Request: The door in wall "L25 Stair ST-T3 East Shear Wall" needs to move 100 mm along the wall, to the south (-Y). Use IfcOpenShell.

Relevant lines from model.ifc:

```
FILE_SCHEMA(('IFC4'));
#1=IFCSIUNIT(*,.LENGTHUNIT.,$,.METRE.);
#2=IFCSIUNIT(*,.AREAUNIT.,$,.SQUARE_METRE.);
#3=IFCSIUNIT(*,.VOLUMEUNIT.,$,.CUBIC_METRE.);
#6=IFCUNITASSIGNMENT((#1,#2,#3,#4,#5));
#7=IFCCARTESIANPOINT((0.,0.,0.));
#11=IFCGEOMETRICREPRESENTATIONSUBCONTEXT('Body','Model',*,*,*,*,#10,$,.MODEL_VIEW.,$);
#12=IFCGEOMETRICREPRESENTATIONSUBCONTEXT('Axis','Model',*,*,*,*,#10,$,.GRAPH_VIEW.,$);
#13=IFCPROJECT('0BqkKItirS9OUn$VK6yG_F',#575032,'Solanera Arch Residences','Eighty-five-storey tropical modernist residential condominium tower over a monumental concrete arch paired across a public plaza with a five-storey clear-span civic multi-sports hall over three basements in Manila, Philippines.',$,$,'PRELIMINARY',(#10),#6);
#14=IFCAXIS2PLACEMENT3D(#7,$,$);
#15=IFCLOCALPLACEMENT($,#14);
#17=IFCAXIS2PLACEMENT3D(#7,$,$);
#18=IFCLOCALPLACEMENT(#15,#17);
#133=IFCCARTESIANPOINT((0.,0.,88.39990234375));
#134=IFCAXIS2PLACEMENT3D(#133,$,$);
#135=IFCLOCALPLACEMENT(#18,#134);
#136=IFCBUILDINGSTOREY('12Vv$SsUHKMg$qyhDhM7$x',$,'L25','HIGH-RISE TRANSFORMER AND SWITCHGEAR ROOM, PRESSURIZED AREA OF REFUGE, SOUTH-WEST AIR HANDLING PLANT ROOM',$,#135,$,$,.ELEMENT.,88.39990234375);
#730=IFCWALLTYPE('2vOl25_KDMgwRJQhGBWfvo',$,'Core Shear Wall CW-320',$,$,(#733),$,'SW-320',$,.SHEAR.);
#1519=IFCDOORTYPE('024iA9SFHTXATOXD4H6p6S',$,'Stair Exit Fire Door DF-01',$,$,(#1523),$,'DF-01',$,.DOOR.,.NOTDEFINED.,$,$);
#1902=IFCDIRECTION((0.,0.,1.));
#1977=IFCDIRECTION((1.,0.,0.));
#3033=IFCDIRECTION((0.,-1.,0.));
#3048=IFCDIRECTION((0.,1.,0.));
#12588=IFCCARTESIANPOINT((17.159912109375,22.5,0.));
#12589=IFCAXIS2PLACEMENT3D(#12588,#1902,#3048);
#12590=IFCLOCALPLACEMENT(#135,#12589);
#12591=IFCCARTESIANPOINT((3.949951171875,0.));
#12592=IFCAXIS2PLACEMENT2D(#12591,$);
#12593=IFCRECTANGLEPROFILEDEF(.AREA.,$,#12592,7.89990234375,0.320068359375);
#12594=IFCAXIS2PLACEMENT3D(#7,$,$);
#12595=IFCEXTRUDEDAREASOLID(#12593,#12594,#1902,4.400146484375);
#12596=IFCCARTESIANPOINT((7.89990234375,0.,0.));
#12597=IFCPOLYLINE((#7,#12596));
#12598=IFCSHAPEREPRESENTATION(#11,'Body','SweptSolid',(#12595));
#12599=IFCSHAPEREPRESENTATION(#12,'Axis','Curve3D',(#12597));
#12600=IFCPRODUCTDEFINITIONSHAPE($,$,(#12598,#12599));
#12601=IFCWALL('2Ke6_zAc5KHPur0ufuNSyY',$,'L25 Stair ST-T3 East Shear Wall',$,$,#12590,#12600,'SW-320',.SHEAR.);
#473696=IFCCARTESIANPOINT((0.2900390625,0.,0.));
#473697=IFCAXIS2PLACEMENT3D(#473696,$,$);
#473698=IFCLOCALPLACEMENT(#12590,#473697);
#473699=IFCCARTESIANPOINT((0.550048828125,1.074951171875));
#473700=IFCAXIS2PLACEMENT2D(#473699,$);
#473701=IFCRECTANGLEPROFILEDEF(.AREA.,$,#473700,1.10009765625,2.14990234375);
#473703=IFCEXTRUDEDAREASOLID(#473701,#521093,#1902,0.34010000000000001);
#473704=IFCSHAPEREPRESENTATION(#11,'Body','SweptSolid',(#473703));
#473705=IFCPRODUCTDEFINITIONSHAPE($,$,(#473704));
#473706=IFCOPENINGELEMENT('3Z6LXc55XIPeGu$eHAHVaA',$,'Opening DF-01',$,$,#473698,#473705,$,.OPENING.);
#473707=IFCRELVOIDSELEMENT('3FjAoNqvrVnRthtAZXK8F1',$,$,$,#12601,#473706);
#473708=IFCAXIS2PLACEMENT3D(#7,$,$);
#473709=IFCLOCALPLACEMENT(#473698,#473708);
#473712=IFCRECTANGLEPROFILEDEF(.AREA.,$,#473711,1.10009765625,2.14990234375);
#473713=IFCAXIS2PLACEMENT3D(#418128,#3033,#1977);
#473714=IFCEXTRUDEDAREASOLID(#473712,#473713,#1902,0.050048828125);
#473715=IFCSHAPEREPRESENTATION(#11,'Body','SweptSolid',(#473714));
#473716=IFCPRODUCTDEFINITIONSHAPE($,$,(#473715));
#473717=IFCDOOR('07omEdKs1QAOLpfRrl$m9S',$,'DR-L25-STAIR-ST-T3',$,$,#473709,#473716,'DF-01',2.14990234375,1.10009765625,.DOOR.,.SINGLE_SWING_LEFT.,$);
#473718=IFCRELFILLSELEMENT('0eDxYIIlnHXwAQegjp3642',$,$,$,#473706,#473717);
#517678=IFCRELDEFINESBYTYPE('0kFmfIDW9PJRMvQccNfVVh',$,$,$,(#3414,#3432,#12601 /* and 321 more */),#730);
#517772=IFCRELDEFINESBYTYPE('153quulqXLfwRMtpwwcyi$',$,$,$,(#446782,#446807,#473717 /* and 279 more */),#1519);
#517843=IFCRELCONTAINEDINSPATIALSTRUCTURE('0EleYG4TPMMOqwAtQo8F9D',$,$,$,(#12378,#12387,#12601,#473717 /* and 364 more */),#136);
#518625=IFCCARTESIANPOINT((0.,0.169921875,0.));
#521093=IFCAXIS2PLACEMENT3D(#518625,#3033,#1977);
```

```python
import ifcopenshell
import ifcopenshell.api.geometry
import ifcopenshell.util.placement

model = ifcopenshell.open("model.ifc")

door = model.by_guid("07omEdKs1QAOLpfRrl$m9S")
opening = door.FillsVoids[0].RelatingOpeningElement
wall = opening.VoidsElements[0].RelatingBuildingElement

wall_matrix = ifcopenshell.util.placement.get_local_placement(wall.ObjectPlacement)
shift = wall_matrix[:3, 0] * -0.1
before = ifcopenshell.util.placement.get_local_placement(door.ObjectPlacement)[:3, 3].copy()

# The door is placed relative to its opening, so it follows when the opening moves.
matrix = ifcopenshell.util.placement.get_local_placement(opening.ObjectPlacement)
matrix[:3, 3] += shift
ifcopenshell.api.geometry.edit_object_placement(
    model, product=opening, matrix=matrix, is_si=False, should_transform_children=True
)

after = ifcopenshell.util.placement.get_local_placement(door.ObjectPlacement)[:3, 3]
print("door moved by", (after - before).round(3) + 0.0)

model.write("model_rev.ifc")
```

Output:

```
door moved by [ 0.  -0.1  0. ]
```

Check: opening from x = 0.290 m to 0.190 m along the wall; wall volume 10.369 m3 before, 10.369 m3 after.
